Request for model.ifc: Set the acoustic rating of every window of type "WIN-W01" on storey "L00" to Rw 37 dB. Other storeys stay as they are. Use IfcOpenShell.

First a look at what the model holds.

```python
import ifcopenshell
import ifcopenshell.util.element

model = ifcopenshell.open("model.ifc")
print(model.schema)
storey = next(s for s in model.by_type("IfcBuildingStorey") if s.Name == "L00")
windows = [e for e in ifcopenshell.util.element.get_decomposition(storey) if e.is_a("IfcWindow")]
seen = {}
for e in windows:
    element_type = ifcopenshell.util.element.get_type(e)
    key = (element_type.Name if element_type != e and element_type else None, ifcopenshell.util.element.get_pset(e, "Pset_WindowCommon", "AcousticRating"))
    seen[key] = seen.get(key, 0) + 1
for (name, value), count in sorted(seen.items(), key=str):
    print(count, "x", name, "|", value)
```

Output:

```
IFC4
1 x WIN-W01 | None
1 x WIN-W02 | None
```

```python
import ifcopenshell
import ifcopenshell.api.pset
import ifcopenshell.util.element

model = ifcopenshell.open("model.ifc")

storey = next(s for s in model.by_type("IfcBuildingStorey") if s.Name == "L00")
windows = [e for e in ifcopenshell.util.element.get_decomposition(storey) if e.is_a("IfcWindow")]

count = 0
for e in windows:
    element_type = ifcopenshell.util.element.get_type(e)
    if element_type in (None, e) or element_type.Name != "WIN-W01":
        continue
    # add_pset returns the element's existing set when there is one.
    pset = ifcopenshell.api.pset.add_pset(model, product=e, name="Pset_WindowCommon")
    ifcopenshell.api.pset.edit_pset(model, pset=pset, properties={"AcousticRating": "Rw 37 dB"})
    count += 1

print(count, "windows updated")

model.write("model_rev.ifc")
```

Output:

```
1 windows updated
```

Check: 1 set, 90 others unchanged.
